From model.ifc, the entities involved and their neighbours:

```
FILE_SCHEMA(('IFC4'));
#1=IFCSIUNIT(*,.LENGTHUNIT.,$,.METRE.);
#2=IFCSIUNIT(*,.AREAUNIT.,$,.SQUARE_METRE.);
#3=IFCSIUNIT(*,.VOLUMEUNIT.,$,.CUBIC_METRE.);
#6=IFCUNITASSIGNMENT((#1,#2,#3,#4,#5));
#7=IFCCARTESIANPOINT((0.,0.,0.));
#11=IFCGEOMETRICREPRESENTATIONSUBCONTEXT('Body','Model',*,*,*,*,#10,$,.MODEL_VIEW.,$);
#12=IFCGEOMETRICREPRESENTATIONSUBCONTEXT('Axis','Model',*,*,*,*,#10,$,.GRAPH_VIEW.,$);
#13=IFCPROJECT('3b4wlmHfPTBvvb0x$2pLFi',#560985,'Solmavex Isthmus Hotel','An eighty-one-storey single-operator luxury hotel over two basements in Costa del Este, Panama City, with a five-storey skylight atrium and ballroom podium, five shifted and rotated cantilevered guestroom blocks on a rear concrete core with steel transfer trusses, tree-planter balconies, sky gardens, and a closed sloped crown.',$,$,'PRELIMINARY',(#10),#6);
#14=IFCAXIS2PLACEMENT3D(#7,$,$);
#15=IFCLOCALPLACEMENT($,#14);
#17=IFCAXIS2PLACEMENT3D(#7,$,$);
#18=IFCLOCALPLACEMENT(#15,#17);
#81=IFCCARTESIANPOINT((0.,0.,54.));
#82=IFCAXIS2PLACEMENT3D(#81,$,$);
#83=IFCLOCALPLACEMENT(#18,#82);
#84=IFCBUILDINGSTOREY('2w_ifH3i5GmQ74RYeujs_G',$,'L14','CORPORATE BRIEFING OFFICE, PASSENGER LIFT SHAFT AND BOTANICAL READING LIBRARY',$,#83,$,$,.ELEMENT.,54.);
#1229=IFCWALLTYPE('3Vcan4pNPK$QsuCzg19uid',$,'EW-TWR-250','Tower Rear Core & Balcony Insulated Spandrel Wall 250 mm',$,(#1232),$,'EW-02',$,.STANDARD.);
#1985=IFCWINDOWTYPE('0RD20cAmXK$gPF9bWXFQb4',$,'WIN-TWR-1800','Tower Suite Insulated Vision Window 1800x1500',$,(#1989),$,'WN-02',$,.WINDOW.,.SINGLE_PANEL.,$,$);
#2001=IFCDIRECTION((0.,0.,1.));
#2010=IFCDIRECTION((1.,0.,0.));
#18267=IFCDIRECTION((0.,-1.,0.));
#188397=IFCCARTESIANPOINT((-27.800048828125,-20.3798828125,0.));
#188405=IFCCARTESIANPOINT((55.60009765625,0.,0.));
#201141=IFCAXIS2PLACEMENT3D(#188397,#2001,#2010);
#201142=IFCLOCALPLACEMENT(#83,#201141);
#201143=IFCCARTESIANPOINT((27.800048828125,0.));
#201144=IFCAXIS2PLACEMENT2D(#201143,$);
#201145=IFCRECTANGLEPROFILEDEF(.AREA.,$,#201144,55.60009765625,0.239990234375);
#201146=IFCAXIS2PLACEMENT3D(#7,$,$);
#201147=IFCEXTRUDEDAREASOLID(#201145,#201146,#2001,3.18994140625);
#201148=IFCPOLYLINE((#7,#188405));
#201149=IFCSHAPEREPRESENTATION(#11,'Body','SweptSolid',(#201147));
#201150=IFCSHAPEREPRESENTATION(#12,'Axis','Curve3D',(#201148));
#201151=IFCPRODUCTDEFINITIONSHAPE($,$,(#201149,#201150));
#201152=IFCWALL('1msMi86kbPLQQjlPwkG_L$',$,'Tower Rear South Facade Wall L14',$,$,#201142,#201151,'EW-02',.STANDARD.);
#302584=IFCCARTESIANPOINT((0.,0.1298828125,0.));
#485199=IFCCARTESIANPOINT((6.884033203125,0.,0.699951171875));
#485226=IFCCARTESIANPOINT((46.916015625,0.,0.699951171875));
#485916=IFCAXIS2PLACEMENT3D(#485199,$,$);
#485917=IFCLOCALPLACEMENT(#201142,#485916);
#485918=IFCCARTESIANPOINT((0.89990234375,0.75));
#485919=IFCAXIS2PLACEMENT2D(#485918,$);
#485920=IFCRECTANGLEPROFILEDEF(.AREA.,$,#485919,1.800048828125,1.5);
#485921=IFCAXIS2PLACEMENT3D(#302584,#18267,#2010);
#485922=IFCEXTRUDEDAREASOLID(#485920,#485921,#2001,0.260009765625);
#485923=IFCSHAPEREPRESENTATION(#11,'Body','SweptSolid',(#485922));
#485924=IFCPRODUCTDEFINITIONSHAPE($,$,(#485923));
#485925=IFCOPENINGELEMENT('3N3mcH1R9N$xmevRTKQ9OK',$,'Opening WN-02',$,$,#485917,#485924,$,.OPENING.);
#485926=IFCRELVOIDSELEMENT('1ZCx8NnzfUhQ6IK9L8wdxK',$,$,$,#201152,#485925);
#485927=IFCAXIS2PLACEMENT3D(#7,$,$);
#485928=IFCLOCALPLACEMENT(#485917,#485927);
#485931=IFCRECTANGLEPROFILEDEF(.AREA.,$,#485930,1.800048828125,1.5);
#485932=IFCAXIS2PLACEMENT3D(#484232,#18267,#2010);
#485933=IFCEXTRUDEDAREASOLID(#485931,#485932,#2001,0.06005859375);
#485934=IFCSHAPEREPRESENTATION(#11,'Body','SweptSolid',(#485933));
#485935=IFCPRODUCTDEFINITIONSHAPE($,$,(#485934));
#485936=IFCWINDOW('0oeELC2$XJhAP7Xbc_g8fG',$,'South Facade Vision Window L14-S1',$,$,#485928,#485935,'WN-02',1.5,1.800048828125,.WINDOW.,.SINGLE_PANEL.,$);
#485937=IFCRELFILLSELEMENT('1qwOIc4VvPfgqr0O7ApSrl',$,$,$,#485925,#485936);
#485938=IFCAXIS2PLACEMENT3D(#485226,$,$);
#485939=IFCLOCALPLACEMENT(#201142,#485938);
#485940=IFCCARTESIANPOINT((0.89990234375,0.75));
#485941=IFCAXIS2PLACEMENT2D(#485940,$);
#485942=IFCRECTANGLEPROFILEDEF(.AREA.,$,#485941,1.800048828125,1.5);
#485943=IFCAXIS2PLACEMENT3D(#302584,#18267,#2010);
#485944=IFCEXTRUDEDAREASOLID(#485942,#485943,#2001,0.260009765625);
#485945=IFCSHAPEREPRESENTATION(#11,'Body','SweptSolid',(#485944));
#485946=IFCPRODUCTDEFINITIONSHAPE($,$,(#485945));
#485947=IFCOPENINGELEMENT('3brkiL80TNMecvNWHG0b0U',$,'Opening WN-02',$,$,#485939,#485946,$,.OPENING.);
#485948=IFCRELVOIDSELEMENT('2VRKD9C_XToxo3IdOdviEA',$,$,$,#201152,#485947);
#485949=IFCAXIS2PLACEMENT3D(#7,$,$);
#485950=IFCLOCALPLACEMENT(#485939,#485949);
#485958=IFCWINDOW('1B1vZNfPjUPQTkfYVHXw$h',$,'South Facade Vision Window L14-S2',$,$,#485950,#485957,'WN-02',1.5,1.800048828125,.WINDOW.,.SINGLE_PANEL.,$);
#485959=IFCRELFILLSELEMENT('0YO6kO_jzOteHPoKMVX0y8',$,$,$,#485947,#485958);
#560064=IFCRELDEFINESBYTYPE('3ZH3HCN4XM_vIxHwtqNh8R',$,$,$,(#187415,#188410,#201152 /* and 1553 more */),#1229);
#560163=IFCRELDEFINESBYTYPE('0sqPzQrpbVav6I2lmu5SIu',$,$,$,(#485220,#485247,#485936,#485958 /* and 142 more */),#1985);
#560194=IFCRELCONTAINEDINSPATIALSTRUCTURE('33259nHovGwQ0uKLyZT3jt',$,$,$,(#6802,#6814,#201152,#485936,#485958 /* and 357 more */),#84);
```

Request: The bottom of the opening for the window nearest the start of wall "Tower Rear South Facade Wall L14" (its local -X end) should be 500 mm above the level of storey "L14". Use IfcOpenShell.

```python
import numpy as np
import ifcopenshell
import ifcopenshell.api.geometry
import ifcopenshell.geom
import ifcopenshell.util.element
import ifcopenshell.util.placement
import ifcopenshell.util.shape
import ifcopenshell.util.unit

model = ifcopenshell.open("model.ifc")
unit_scale = ifcopenshell.util.unit.calculate_unit_scale(model)

window = model.by_guid("0oeELC2$XJhAP7Xbc_g8fG")
opening = window.FillsVoids[0].RelatingOpeningElement
storey = ifcopenshell.util.element.get_container(window, ifc_class="IfcBuildingStorey")
level = ifcopenshell.util.placement.get_local_placement(storey.ObjectPlacement)[2, 3]

# The opening's origin need not be at the sill, so measure its lowest point.
shape = ifcopenshell.geom.create_shape(ifcopenshell.geom.settings(), opening)
bottom = ifcopenshell.util.shape.get_shape_bottom_elevation(shape, shape.geometry) / unit_scale
dz = level + 0.5 - bottom

shift = np.array([0.0, 0.0, dz])
# The window is placed relative to its opening, so it follows when the opening moves.
matrix = ifcopenshell.util.placement.get_local_placement(opening.ObjectPlacement)
matrix[:3, 3] += shift
ifcopenshell.api.geometry.edit_object_placement(
    model, product=opening, matrix=matrix, is_si=False, should_transform_children=True
)

print(f"moved by {dz * unit_scale:+.3f} m")

model.write("model_updated.ifc")
```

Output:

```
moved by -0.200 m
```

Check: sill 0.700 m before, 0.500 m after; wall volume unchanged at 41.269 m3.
